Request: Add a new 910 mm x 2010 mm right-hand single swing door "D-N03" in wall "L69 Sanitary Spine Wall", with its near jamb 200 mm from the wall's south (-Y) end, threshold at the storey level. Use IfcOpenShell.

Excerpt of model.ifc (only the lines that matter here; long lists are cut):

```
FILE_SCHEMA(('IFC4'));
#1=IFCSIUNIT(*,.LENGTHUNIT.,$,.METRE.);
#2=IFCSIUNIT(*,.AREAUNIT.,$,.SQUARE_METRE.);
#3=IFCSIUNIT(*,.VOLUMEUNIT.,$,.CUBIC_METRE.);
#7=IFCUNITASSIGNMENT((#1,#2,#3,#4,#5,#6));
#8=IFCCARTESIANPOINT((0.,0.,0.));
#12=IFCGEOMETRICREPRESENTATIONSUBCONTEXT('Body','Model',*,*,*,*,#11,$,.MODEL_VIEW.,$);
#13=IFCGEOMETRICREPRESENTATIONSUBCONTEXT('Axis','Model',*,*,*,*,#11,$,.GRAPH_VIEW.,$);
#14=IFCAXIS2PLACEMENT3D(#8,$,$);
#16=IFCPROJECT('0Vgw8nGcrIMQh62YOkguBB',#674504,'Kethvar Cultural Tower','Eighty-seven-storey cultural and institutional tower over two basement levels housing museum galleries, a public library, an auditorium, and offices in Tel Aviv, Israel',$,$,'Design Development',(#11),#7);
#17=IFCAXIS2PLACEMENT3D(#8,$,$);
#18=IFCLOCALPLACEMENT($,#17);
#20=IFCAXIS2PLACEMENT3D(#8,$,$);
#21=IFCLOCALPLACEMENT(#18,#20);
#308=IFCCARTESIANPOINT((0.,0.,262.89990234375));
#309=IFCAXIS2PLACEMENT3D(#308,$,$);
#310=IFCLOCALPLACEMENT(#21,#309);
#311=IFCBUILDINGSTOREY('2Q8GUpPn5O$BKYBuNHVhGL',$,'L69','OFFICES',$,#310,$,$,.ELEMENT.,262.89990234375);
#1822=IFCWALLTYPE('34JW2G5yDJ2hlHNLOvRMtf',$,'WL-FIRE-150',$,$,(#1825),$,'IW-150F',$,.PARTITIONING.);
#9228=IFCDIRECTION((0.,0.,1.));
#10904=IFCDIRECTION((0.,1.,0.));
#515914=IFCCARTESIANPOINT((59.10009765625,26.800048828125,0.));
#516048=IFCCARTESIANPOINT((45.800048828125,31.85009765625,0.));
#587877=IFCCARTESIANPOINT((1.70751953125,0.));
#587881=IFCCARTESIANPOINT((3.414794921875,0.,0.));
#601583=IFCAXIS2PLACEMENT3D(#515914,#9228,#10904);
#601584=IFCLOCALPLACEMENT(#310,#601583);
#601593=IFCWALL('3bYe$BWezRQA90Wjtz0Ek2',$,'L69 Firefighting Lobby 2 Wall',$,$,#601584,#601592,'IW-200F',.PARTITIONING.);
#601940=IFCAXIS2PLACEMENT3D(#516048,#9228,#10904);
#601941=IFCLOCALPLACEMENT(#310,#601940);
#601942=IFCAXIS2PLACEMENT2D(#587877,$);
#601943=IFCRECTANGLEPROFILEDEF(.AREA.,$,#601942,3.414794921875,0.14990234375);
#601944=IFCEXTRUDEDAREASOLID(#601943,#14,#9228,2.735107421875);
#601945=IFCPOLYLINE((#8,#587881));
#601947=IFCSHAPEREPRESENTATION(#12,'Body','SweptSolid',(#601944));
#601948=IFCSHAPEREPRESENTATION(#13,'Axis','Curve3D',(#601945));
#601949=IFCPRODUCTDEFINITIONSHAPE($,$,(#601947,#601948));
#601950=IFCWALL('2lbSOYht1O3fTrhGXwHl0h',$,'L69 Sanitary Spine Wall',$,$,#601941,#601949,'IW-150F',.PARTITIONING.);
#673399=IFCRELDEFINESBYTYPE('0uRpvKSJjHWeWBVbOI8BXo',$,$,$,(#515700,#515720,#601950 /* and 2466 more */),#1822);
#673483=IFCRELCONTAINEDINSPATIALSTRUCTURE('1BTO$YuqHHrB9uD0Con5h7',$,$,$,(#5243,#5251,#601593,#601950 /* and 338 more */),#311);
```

```python
import numpy as np
import ifcopenshell
import ifcopenshell.api.feature
import ifcopenshell.api.geometry
import ifcopenshell.api.root
import ifcopenshell.api.spatial
import ifcopenshell.geom
import ifcopenshell.util.element
import ifcopenshell.util.placement
import ifcopenshell.util.representation
import ifcopenshell.util.shape
import ifcopenshell.util.unit

model = ifcopenshell.open("model.ifc")
unit_scale = ifcopenshell.util.unit.calculate_unit_scale(model)
settings = ifcopenshell.geom.settings()


def volume(element):
    """Net volume in cubic metres, openings subtracted."""
    shape = ifcopenshell.geom.create_shape(settings, element)
    return ifcopenshell.util.shape.get_volume(shape.geometry)


wall = model.by_id(601950)
storey = ifcopenshell.util.element.get_container(wall, ifc_class="IfcBuildingStorey")
context = ifcopenshell.util.representation.get_context(model, "Model", "Body", "MODEL_VIEW")
before = volume(wall)

width, height, from_end, sill = 0.91, 2.01, 0.2, 0.0  # metres

# The wall runs along its own X axis, and the end named is its -X end.
wall_shape = ifcopenshell.geom.create_shape(settings, wall)
x, y, z = ifcopenshell.util.shape.get_vertices(wall_shape.geometry).T
start = x.min() + from_end
face, thickness = float(y.min()), float(y.max() - y.min())
wall_matrix = ifcopenshell.util.placement.get_local_placement(wall.ObjectPlacement)
level = ifcopenshell.util.placement.get_local_placement(storey.ObjectPlacement)[2, 3]


def in_wall(x, y):
    """Placement at x, y metres in the wall's axes, at sill height."""
    matrix = wall_matrix.copy()
    matrix[:, 3] = wall_matrix @ np.array([x / unit_scale, y / unit_scale, 0.0, 1.0])
    matrix[2, 3] = level + sill / unit_scale
    return matrix


# Opening: a box that overshoots both wall faces by 50 mm.
opening = ifcopenshell.api.root.create_entity(model, ifc_class="IfcOpeningElement", predefined_type="OPENING")
box = ifcopenshell.api.geometry.add_wall_representation(
    model, context=context, length=width, height=height, thickness=thickness + 0.1
)
ifcopenshell.api.geometry.assign_representation(model, product=opening, representation=box)
ifcopenshell.api.geometry.edit_object_placement(model, product=opening, matrix=in_wall(start, face - 0.05), is_si=False)
ifcopenshell.api.feature.add_feature(model, feature=opening, element=wall)

door = ifcopenshell.api.root.create_entity(model, ifc_class="IfcDoor", name="D-N03", predefined_type="DOOR")
door.OverallWidth, door.OverallHeight = width / unit_scale, height / unit_scale
door.OperationType = "SINGLE_SWING_RIGHT"
body = ifcopenshell.api.geometry.add_door_representation(
    model,
    context=context,
    overall_width=door.OverallWidth,
    overall_height=door.OverallHeight,
    operation_type="SINGLE_SWING_RIGHT",
    lining_properties={"LiningDepth": thickness / unit_scale, "ThresholdDepth": thickness / unit_scale},
)
ifcopenshell.api.geometry.assign_representation(model, product=door, representation=body)
ifcopenshell.api.spatial.assign_container(model, products=[door], relating_structure=storey)
ifcopenshell.api.feature.add_filling(model, opening=opening, element=door)

# The lining spans the wall, so the door starts at the wall face.
ifcopenshell.api.geometry.edit_object_placement(model, product=door, matrix=in_wall(start, face), is_si=False)

after = volume(wall)

print(f"wall volume {before:.3f} -> {after:.3f} m3")

model.write("model-out.ifc")
```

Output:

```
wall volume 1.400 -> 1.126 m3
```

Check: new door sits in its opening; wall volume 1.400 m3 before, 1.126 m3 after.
